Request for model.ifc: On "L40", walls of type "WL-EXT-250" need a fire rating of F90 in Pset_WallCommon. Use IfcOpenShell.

First a look at what the model holds.

```python
import ifcopenshell
import ifcopenshell.util.element

model = ifcopenshell.open("model.ifc")
print(model.schema)
storey = next(s for s in model.by_type("IfcBuildingStorey") if s.Name == "L40")
walls = [e for e in ifcopenshell.util.element.get_decomposition(storey) if e.is_a("IfcWall")]
seen = {}
for e in walls:
    element_type = ifcopenshell.util.element.get_type(e)
    key = (element_type.Name if element_type != e and element_type else None, ifcopenshell.util.element.get_pset(e, "Pset_WallCommon", "FireRating"))
    seen[key] = seen.get(key, 0) + 1
for (name, value), count in sorted(seen.items(), key=str):
    print(count, "x", name, "|", value)
```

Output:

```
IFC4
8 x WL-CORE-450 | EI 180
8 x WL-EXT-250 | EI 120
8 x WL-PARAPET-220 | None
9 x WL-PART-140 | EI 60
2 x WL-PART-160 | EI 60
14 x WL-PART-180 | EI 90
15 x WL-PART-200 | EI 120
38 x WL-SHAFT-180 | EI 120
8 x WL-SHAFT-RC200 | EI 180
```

```python
import ifcopenshell
import ifcopenshell.api.pset
import ifcopenshell.util.element

model = ifcopenshell.open("model.ifc")

storey = next(s for s in model.by_type("IfcBuildingStorey") if s.Name == "L40")
walls = [e for e in ifcopenshell.util.element.get_decomposition(storey) if e.is_a("IfcWall")]

count = 0
for e in walls:
    element_type = ifcopenshell.util.element.get_type(e)
    if element_type in (None, e) or element_type.Name != "WL-EXT-250":
        continue
    found = ifcopenshell.util.element.get_pset(e, "Pset_WallCommon", should_inherit=False)
    if found:
        pset = model.by_id(found["id"])
        if len(ifcopenshell.util.element.get_elements_by_pset(pset)) > 1:
            pset = ifcopenshell.api.pset.unshare_pset(model, products=[e], pset=pset)[0]
    else:
        pset = ifcopenshell.api.pset.add_pset(model, product=e, name="Pset_WallCommon")
    ifcopenshell.api.pset.edit_pset(model, pset=pset, properties={"FireRating": "F90"})
    count += 1

print(count, "walls updated")

model.write("model_v2.ifc")
```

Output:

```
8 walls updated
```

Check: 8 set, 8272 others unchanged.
